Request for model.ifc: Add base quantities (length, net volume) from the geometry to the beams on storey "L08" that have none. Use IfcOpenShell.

First a look at what the model holds.

```python
import ifcopenshell
import ifcopenshell.util.element
import ifcopenshell.util.unit

model = ifcopenshell.open("model.ifc")
print(model.schema)
for unit_type in ("LENGTHUNIT", "AREAUNIT", "VOLUMEUNIT"):
    print(unit_type, ifcopenshell.util.unit.calculate_unit_scale(model, unit_type))
storey = next(s for s in model.by_type("IfcBuildingStorey") if s.Name == "L08")
beams = [e for e in ifcopenshell.util.element.get_decomposition(storey) if e.is_a("IfcBeam")]
for e in sorted(beams, key=lambda e: e.id()):
    print(e.id(), e.is_a(), e.Name, list(ifcopenshell.util.element.get_psets(e, qtos_only=True)), sep=" | ")
```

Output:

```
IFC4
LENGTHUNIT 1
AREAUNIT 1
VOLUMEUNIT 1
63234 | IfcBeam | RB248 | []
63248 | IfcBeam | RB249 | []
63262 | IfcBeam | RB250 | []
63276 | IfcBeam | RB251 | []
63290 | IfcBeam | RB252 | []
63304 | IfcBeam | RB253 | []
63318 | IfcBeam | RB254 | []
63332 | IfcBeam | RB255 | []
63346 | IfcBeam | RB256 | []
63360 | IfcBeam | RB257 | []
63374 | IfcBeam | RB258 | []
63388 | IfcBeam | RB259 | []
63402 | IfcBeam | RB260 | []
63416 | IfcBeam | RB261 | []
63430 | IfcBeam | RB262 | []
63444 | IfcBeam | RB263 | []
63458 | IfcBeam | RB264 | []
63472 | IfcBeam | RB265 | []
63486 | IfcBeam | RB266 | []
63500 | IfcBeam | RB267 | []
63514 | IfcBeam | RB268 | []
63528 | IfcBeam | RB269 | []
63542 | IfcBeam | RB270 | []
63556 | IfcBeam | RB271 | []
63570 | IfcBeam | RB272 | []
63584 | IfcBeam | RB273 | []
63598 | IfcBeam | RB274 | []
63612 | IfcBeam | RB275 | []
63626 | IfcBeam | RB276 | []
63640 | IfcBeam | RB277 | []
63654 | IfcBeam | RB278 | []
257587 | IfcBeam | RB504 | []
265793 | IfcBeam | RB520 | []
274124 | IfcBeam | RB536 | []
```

```python
import ifcopenshell
import ifcopenshell.api.pset
import ifcopenshell.geom
import ifcopenshell.util.element
import ifcopenshell.util.shape
import ifcopenshell.util.unit

model = ifcopenshell.open("model.ifc")
unit_scale = ifcopenshell.util.unit.calculate_unit_scale(model)
volume_scale = ifcopenshell.util.unit.calculate_unit_scale(model, "VOLUMEUNIT")
settings = ifcopenshell.geom.settings()

storey = next(s for s in model.by_type("IfcBuildingStorey") if s.Name == "L08")
beams = [e for e in ifcopenshell.util.element.get_decomposition(storey) if e.is_a("IfcBeam")]

for e in sorted(beams, key=lambda e: e.id()):
    if ifcopenshell.util.element.get_psets(e, qtos_only=True, should_inherit=False):
        continue
    # Geometry comes back in metres, in the element's own axes.
    shape = ifcopenshell.geom.create_shape(settings, e)
    values = {
        "Length": ifcopenshell.util.shape.get_max_xyz(shape.geometry) / unit_scale,
        "NetVolume": ifcopenshell.util.shape.get_volume(shape.geometry) / volume_scale,
    }
    qto = ifcopenshell.api.pset.add_qto(model, product=e, name="Qto_BeamBaseQuantities")
    ifcopenshell.api.pset.edit_qto(model, qto=qto, properties=values)
    print(e.id(), {k: round(v, 3) for k, v in values.items()})

model.write("model-out.ifc")
```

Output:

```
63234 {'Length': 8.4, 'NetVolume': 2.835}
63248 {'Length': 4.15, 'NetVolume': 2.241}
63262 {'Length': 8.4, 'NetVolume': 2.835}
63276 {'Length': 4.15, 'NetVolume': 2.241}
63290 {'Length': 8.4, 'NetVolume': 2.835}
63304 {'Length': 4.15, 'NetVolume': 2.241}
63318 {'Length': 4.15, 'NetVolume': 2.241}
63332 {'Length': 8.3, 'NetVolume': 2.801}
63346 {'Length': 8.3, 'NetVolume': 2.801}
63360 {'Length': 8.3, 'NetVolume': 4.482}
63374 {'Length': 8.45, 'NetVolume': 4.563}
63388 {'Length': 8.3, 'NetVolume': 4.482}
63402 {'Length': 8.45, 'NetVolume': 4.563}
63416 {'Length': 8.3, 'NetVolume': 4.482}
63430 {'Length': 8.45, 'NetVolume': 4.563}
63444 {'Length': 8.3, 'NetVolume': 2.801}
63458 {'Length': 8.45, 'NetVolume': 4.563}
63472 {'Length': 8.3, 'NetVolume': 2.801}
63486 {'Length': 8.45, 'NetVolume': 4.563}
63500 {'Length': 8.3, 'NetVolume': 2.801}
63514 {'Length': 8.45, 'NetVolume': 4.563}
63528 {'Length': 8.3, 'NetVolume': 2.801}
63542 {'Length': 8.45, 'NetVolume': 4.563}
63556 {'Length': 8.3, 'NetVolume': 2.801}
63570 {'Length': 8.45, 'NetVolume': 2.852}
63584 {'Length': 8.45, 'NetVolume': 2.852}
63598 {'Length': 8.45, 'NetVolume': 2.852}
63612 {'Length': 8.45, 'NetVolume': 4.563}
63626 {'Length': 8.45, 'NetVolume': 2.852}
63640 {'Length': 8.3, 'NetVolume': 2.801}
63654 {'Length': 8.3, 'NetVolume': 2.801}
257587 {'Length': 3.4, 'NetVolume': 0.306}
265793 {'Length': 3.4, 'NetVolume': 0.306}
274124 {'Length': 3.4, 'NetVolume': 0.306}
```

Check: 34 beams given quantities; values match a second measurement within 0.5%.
